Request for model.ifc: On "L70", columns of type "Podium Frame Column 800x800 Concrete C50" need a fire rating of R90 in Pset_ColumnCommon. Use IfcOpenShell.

First a look at what the model holds.

```python
import ifcopenshell
import ifcopenshell.util.element

model = ifcopenshell.open("model.ifc")
print(model.schema)
storey = next(s for s in model.by_type("IfcBuildingStorey") if s.Name == "L70")
columns = [e for e in ifcopenshell.util.element.get_decomposition(storey) if e.is_a("IfcColumn")]
seen = {}
for e in columns:
    element_type = ifcopenshell.util.element.get_type(e)
    key = (element_type.Name if element_type != e and element_type else None, ifcopenshell.util.element.get_pset(e, "Pset_ColumnCommon", "FireRating"))
    seen[key] = seen.get(key, 0) + 1
for (name, value), count in sorted(seen.items(), key=str):
    print(count, "x", name, "|", value)
```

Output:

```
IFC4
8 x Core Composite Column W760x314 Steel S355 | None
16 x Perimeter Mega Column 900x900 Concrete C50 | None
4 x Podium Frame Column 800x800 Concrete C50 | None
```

```python
import ifcopenshell
import ifcopenshell.api.pset
import ifcopenshell.util.element

model = ifcopenshell.open("model.ifc")

storey = next(s for s in model.by_type("IfcBuildingStorey") if s.Name == "L70")
columns = [e for e in ifcopenshell.util.element.get_decomposition(storey) if e.is_a("IfcColumn")]

count = 0
for e in columns:
    element_type = ifcopenshell.util.element.get_type(e)
    if element_type in (None, e) or element_type.Name != "Podium Frame Column 800x800 Concrete C50":
        continue
    found = ifcopenshell.util.element.get_pset(e, "Pset_ColumnCommon", should_inherit=False)
    if found:
        pset = model.by_id(found["id"])
        if len(ifcopenshell.util.element.get_elements_by_pset(pset)) > 1:
            pset = ifcopenshell.api.pset.unshare_pset(model, products=[e], pset=pset)[0]
    else:
        pset = ifcopenshell.api.pset.add_pset(model, product=e, name="Pset_ColumnCommon")
    ifcopenshell.api.pset.edit_pset(model, pset=pset, properties={"FireRating": "R90"})
    count += 1

print(count, "columns updated")

model.write("model-out.ifc")
```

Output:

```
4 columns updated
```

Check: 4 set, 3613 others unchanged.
